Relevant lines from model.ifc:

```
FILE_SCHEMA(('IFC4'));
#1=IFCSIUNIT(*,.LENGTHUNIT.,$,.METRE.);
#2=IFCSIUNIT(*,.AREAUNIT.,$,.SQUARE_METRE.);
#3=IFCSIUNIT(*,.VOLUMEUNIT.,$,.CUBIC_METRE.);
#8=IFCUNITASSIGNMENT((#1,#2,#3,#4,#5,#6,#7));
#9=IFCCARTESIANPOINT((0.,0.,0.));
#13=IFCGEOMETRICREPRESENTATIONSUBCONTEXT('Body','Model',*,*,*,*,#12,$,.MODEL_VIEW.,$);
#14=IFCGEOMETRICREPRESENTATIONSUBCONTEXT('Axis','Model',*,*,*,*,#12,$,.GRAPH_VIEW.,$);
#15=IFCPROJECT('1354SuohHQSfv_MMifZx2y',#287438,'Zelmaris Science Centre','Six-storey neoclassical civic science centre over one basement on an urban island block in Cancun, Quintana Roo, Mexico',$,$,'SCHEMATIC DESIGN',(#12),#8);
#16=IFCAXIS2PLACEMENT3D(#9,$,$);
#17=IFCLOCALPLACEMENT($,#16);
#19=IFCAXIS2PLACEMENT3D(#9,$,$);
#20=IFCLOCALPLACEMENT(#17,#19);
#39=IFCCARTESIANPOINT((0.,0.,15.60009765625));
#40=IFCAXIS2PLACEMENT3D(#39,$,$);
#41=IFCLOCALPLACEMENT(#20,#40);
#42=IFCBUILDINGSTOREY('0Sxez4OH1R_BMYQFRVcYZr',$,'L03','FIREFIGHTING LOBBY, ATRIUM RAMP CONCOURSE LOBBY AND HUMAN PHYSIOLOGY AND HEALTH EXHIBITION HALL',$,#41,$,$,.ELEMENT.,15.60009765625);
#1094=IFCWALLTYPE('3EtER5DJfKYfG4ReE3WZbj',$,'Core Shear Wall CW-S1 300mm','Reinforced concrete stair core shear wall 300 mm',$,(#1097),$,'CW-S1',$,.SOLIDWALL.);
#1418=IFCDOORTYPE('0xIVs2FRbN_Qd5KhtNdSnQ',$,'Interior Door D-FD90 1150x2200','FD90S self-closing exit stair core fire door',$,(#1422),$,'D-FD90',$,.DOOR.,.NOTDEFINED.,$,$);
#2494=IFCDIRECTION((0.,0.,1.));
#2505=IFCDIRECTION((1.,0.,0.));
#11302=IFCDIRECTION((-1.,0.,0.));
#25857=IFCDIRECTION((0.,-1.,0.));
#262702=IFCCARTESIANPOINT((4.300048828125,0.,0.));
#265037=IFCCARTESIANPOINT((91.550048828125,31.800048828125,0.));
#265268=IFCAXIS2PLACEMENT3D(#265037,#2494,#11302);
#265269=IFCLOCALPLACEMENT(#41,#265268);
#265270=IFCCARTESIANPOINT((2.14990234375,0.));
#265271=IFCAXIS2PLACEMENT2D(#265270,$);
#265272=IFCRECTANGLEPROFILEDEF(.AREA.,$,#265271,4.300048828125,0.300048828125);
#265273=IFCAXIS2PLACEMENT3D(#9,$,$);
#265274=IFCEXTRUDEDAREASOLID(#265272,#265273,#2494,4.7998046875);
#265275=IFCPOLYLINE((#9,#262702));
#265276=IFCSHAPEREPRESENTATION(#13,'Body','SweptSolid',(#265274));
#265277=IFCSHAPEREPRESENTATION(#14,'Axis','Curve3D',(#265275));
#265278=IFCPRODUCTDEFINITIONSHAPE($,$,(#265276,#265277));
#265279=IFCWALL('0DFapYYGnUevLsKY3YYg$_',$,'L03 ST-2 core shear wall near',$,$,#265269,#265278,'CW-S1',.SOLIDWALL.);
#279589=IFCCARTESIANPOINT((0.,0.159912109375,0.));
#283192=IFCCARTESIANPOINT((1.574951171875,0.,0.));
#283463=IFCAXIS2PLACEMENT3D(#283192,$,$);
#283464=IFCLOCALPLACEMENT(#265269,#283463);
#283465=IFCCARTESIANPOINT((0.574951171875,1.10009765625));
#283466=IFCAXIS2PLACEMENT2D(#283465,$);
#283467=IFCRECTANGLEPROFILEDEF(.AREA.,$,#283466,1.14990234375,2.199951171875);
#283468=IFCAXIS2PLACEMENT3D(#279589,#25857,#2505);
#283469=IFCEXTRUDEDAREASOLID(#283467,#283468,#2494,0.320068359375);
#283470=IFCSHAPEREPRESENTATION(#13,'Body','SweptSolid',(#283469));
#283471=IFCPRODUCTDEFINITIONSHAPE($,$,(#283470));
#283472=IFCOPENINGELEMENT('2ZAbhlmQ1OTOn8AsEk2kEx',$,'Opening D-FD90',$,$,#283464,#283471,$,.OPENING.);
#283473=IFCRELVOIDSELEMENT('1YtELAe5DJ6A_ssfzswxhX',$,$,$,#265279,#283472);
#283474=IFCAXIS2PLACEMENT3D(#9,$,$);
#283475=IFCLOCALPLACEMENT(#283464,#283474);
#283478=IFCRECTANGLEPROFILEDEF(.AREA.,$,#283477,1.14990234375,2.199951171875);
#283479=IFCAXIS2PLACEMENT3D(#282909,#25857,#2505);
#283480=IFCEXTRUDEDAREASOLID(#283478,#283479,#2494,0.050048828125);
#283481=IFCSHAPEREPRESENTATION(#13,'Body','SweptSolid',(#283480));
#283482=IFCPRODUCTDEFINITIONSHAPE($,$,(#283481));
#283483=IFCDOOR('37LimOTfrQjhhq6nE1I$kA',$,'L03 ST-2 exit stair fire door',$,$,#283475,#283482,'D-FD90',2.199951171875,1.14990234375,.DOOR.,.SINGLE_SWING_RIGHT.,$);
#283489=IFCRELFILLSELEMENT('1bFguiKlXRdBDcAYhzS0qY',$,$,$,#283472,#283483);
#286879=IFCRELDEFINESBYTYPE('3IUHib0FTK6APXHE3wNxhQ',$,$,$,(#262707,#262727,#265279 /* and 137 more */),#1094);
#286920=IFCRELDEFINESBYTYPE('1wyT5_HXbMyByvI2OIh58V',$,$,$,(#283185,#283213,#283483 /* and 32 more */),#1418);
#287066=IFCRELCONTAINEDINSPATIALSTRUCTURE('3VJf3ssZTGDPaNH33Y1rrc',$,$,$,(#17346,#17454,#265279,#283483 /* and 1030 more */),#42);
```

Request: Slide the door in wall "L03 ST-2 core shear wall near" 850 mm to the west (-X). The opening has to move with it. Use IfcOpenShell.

```python
import ifcopenshell
import ifcopenshell.api.geometry
import ifcopenshell.util.placement
import ifcopenshell.util.unit

model = ifcopenshell.open("model.ifc")
unit_scale = ifcopenshell.util.unit.calculate_unit_scale(model)

door = model.by_guid("37LimOTfrQjhhq6nE1I$kA")
opening = door.FillsVoids[0].RelatingOpeningElement
wall = opening.VoidsElements[0].RelatingBuildingElement

wall_matrix = ifcopenshell.util.placement.get_local_placement(wall.ObjectPlacement)
shift = wall_matrix[:3, 0] * 0.85 / unit_scale
before = ifcopenshell.util.placement.get_local_placement(door.ObjectPlacement)[:3, 3].copy()

# The door is placed relative to its opening, so it follows when the opening moves.
matrix = ifcopenshell.util.placement.get_local_placement(opening.ObjectPlacement)
matrix[:3, 3] += shift
ifcopenshell.api.geometry.edit_object_placement(
    model, product=opening, matrix=matrix, is_si=False, should_transform_children=True
)

after = ifcopenshell.util.placement.get_local_placement(door.ObjectPlacement)[:3, 3]
print("door moved by", (after - before).round(3) + 0.0)

model.write("model_edited.ifc")
```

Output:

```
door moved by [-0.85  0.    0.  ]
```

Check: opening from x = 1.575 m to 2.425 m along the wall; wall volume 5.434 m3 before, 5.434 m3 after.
